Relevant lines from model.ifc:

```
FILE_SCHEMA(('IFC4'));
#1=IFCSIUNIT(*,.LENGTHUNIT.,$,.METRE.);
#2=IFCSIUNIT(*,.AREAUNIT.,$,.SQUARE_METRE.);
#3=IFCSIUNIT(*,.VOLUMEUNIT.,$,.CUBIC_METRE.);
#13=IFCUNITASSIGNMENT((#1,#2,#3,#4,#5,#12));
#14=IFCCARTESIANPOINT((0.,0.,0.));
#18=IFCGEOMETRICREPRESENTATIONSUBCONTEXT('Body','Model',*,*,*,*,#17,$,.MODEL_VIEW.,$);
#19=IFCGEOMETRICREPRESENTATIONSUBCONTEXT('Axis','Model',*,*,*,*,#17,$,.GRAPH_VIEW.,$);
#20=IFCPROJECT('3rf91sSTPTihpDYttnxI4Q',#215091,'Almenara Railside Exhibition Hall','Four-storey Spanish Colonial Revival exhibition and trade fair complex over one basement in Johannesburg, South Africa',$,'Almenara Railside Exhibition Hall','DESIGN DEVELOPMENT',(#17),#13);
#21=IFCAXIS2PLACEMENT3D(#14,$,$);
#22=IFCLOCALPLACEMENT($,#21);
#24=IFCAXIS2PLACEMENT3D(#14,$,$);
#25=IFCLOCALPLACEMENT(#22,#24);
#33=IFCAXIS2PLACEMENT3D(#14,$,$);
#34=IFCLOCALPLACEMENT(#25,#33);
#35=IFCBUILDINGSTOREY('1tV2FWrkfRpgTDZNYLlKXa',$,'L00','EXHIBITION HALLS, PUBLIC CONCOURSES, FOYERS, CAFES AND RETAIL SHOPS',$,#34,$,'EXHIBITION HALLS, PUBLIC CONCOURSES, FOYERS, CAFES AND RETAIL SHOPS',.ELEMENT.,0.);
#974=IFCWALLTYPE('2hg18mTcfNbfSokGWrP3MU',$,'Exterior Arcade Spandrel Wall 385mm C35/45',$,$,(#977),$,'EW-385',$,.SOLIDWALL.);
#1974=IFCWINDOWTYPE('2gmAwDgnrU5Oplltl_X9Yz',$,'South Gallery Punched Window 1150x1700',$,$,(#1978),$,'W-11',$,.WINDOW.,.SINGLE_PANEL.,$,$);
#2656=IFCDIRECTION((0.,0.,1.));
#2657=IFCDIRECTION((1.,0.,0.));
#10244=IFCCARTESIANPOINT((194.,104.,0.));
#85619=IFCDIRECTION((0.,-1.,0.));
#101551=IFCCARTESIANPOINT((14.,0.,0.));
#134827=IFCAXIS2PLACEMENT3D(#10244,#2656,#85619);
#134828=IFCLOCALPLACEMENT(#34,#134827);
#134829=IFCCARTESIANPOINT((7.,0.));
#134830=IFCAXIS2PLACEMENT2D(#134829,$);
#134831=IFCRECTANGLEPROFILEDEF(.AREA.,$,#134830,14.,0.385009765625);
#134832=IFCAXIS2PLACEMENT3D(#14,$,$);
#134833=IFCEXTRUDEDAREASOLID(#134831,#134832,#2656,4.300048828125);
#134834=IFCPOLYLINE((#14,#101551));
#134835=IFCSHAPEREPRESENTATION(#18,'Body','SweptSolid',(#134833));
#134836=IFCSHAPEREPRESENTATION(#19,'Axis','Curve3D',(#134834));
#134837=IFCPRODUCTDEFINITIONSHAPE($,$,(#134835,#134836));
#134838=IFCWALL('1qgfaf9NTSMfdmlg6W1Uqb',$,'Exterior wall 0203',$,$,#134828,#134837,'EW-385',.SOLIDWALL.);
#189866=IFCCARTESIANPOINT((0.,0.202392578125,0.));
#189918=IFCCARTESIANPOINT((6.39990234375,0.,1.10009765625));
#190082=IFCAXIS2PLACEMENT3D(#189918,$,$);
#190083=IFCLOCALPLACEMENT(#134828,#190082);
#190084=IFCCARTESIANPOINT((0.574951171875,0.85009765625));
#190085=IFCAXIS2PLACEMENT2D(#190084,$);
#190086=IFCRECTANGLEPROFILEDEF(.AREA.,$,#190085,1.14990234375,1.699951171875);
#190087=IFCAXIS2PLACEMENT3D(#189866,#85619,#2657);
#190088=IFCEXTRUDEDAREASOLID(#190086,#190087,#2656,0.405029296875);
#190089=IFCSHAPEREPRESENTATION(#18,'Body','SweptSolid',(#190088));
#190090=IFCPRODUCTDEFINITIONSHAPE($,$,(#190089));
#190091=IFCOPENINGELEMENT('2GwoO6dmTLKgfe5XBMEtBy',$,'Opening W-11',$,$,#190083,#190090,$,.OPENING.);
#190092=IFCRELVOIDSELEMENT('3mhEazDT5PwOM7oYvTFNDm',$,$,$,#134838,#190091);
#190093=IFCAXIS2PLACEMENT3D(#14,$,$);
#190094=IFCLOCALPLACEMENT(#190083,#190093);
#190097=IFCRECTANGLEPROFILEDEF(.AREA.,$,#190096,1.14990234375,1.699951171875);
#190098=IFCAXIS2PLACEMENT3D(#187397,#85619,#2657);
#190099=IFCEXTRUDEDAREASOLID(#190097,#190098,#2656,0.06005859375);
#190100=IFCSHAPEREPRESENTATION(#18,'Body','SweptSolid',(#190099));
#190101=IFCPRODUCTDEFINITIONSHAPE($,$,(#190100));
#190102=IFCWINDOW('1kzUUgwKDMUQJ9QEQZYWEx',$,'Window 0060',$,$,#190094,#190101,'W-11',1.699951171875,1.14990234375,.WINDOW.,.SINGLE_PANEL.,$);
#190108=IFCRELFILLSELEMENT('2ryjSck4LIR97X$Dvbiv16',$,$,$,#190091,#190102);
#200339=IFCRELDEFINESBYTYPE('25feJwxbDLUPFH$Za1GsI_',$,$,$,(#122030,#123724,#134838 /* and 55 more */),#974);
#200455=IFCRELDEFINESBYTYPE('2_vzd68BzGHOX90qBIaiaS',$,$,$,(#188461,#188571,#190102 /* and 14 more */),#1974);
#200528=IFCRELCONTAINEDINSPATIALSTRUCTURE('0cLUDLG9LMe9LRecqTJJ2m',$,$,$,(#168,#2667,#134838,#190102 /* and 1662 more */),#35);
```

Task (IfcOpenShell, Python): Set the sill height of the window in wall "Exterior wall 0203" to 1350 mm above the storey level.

```python
import numpy as np
import ifcopenshell
import ifcopenshell.api.geometry
import ifcopenshell.geom
import ifcopenshell.util.element
import ifcopenshell.util.placement
import ifcopenshell.util.shape
import ifcopenshell.util.unit

model = ifcopenshell.open("model.ifc")
unit_scale = ifcopenshell.util.unit.calculate_unit_scale(model)

window = model.by_guid("1kzUUgwKDMUQJ9QEQZYWEx")
opening = window.FillsVoids[0].RelatingOpeningElement
storey = ifcopenshell.util.element.get_container(window, ifc_class="IfcBuildingStorey")
level = ifcopenshell.util.placement.get_local_placement(storey.ObjectPlacement)[2, 3]

# The opening's origin need not be at the sill, so measure its lowest point.
shape = ifcopenshell.geom.create_shape(ifcopenshell.geom.settings(), opening)
bottom = ifcopenshell.util.shape.get_shape_bottom_elevation(shape, shape.geometry) / unit_scale
dz = level + 1.35 - bottom

shift = np.array([0.0, 0.0, dz])
# The window is placed relative to its opening, so it follows when the opening moves.
matrix = ifcopenshell.util.placement.get_local_placement(opening.ObjectPlacement)
matrix[:3, 3] += shift
ifcopenshell.api.geometry.edit_object_placement(
    model, product=opening, matrix=matrix, is_si=False, should_transform_children=True
)

print(f"moved by {dz * unit_scale:+.3f} m")

model.write("model_updated.ifc")
```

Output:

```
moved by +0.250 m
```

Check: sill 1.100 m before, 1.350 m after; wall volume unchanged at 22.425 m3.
